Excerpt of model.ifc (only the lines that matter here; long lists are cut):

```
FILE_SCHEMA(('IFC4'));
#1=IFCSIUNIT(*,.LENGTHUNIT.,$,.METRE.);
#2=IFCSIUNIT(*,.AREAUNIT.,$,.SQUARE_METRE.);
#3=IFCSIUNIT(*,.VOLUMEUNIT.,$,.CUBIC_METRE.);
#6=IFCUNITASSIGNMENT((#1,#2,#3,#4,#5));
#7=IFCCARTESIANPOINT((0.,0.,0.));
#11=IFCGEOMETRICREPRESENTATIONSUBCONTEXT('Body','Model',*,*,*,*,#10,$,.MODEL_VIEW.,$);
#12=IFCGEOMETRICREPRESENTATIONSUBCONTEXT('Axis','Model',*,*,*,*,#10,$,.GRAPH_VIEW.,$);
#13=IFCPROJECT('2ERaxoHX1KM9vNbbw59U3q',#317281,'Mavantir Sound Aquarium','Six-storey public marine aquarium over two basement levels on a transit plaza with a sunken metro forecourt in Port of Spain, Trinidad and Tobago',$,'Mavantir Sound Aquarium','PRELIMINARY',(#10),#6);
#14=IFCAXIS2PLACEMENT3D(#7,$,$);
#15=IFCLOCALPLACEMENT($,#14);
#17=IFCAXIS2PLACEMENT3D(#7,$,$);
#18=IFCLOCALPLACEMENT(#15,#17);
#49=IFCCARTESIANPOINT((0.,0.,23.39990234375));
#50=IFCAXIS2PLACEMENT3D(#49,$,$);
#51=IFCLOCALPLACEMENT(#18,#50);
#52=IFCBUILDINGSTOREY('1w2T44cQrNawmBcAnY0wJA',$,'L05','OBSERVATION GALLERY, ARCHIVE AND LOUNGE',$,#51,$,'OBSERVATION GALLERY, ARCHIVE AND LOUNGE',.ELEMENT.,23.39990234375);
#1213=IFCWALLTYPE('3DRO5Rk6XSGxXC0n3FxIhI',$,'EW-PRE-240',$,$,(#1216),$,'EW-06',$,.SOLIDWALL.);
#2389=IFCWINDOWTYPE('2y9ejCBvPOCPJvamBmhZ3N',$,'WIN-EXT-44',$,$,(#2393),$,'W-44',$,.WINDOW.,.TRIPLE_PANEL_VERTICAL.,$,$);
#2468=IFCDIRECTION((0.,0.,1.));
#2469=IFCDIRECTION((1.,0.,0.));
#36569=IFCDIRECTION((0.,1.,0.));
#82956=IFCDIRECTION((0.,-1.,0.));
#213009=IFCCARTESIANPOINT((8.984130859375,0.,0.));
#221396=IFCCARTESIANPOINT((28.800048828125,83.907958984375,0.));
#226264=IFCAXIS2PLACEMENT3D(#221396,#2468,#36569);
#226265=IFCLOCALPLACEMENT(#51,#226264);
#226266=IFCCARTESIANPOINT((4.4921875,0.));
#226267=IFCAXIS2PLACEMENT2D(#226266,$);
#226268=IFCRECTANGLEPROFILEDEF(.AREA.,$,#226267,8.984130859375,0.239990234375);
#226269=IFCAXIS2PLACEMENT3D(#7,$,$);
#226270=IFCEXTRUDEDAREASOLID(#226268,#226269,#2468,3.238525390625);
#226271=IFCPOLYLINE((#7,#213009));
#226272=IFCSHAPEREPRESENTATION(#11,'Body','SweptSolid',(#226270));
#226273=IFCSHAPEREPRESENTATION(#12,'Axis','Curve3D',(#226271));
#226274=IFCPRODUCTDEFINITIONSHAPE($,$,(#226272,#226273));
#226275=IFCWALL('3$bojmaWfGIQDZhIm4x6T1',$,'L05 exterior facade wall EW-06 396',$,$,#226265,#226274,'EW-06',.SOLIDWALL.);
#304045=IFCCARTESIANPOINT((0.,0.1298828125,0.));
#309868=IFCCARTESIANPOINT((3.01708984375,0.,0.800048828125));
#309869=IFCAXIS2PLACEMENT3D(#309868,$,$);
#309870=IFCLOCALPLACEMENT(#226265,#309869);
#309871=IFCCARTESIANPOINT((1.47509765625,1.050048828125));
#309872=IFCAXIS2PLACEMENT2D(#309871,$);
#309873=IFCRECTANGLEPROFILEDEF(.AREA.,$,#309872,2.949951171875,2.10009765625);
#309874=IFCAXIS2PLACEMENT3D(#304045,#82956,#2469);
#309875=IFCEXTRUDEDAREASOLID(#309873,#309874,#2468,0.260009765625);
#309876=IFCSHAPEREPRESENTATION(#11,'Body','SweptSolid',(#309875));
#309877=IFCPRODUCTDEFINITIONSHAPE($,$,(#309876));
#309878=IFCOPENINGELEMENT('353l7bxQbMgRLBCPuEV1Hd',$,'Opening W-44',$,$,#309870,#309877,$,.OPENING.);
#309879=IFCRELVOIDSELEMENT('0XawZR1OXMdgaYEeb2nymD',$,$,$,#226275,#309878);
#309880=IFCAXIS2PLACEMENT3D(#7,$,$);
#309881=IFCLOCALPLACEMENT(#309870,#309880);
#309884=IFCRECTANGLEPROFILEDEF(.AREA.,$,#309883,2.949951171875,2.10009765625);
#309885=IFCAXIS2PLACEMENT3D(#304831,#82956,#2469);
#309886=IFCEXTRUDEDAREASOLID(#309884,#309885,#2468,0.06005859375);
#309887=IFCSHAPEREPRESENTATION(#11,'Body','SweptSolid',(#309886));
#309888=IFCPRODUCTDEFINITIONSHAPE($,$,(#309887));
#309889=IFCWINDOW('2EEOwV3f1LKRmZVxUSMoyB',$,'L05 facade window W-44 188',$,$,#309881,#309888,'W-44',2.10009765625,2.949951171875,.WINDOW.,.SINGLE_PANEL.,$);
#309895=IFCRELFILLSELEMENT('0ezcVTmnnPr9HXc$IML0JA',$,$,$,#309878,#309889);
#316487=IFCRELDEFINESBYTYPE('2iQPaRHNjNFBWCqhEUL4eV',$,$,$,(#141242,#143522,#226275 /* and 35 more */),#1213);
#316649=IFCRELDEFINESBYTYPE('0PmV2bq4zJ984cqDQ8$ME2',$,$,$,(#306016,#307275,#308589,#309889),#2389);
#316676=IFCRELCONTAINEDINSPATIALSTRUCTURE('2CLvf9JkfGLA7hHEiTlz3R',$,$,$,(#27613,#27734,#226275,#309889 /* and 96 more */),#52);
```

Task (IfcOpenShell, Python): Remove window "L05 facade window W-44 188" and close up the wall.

```python
import ifcopenshell
import ifcopenshell.api.feature
import ifcopenshell.api.root
import ifcopenshell.geom
import ifcopenshell.util.shape

model = ifcopenshell.open("model.ifc")
settings = ifcopenshell.geom.settings()


def volume(element):
    """Net volume in cubic metres, openings subtracted."""
    shape = ifcopenshell.geom.create_shape(settings, element)
    return ifcopenshell.util.shape.get_volume(shape.geometry)


window = model.by_guid("2EEOwV3f1LKRmZVxUSMoyB")
opening = window.FillsVoids[0].RelatingOpeningElement
wall = opening.VoidsElements[0].RelatingBuildingElement
before = volume(wall)

ifcopenshell.api.root.remove_product(model, product=window)
ifcopenshell.api.feature.remove_feature(model, feature=opening)

after = volume(wall)

print(f"wall volume {before:.3f} -> {after:.3f} m3")

model.write("model_updated.ifc")
```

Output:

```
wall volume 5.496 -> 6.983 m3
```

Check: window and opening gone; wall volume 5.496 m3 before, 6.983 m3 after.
